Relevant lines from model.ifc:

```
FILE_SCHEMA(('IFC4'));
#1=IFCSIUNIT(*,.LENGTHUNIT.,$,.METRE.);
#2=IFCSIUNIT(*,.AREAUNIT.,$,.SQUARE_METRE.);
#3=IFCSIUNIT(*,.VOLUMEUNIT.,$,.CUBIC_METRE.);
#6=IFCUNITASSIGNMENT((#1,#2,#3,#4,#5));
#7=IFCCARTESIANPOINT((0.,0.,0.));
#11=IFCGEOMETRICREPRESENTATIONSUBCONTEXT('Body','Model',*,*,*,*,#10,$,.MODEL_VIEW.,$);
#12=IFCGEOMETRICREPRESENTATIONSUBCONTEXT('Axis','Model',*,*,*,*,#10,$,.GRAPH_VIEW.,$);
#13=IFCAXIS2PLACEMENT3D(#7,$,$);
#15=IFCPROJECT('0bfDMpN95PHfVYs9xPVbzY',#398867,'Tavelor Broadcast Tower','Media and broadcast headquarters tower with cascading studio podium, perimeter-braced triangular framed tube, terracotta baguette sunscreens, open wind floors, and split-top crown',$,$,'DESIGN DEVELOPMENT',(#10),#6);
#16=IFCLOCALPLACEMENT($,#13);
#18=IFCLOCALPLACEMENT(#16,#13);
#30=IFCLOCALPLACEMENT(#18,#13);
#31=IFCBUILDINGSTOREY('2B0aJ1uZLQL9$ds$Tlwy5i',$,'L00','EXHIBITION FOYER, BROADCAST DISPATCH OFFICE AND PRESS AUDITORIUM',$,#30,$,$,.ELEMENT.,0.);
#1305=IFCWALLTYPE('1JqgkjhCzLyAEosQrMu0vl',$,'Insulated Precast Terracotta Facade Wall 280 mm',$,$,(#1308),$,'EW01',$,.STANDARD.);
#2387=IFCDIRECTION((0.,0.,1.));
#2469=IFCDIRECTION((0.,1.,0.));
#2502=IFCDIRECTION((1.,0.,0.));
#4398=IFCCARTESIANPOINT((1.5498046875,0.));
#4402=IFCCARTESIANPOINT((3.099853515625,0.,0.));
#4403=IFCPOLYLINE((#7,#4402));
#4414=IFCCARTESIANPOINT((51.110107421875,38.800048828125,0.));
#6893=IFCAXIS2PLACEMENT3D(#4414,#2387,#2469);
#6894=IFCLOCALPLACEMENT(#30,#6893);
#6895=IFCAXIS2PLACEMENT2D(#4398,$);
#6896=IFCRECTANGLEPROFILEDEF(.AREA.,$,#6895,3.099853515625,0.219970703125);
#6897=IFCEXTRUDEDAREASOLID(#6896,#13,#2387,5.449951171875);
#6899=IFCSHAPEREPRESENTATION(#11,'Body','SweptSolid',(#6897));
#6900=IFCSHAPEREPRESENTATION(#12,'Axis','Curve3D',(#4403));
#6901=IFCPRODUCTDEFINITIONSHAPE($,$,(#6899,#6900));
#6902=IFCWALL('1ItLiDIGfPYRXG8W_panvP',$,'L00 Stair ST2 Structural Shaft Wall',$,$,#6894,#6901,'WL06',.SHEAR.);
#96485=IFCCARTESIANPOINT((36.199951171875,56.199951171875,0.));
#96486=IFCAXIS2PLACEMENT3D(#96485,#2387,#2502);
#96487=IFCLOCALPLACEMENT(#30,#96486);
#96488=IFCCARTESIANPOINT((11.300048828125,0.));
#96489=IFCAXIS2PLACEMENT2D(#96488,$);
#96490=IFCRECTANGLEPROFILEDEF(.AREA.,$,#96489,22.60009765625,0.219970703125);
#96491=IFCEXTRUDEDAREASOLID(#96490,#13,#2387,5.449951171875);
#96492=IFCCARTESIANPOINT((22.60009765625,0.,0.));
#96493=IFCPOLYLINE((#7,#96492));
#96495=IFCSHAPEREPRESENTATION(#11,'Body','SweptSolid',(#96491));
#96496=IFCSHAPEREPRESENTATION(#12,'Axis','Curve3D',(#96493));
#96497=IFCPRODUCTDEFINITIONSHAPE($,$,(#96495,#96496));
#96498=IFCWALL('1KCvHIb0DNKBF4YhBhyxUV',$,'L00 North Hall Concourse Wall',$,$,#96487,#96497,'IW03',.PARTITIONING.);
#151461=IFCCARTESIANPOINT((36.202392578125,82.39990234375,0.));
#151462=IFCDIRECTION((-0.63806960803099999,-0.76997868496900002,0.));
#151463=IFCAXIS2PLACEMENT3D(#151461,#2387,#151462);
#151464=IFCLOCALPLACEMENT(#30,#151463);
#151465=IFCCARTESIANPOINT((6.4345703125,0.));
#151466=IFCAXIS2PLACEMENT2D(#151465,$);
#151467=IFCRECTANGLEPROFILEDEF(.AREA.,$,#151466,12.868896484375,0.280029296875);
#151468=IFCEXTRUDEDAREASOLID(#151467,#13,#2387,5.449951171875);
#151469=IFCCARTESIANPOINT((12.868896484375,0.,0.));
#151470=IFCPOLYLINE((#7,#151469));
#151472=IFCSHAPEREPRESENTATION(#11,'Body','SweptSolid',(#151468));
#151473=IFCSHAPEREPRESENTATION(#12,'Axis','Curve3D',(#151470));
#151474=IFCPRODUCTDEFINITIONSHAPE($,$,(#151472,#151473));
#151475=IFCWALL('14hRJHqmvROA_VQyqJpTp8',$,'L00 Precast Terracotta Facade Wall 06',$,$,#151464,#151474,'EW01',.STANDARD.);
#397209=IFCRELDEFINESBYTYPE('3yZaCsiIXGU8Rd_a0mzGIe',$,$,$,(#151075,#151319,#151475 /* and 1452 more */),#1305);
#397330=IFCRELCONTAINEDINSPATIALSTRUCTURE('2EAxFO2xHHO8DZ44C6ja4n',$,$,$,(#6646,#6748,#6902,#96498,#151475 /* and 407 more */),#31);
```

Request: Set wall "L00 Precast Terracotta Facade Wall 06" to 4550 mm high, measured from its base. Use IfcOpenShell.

```python
import ifcopenshell
import ifcopenshell.geom
import ifcopenshell.util.representation
import ifcopenshell.util.shape

model = ifcopenshell.open("model.ifc")
settings = ifcopenshell.geom.settings()


def volume(element):
    """Net volume in cubic metres, openings subtracted."""
    shape = ifcopenshell.geom.create_shape(settings, element)
    return ifcopenshell.util.shape.get_volume(shape.geometry)


wall = model.by_guid("14hRJHqmvROA_VQyqJpTp8")
before = volume(wall)

body = ifcopenshell.util.representation.get_representation(wall, "Model", "Body")
solid = body.Items[0]
old_height = solid.Depth
solid.Depth = 4.55
after = volume(wall)

print(f"height {old_height:g} -> {solid.Depth:g}, volume {before:.3f} -> {after:.3f} m3")

model.write("model_rev.ifc")
```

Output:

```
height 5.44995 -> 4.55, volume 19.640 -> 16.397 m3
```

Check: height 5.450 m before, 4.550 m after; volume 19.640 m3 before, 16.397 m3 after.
